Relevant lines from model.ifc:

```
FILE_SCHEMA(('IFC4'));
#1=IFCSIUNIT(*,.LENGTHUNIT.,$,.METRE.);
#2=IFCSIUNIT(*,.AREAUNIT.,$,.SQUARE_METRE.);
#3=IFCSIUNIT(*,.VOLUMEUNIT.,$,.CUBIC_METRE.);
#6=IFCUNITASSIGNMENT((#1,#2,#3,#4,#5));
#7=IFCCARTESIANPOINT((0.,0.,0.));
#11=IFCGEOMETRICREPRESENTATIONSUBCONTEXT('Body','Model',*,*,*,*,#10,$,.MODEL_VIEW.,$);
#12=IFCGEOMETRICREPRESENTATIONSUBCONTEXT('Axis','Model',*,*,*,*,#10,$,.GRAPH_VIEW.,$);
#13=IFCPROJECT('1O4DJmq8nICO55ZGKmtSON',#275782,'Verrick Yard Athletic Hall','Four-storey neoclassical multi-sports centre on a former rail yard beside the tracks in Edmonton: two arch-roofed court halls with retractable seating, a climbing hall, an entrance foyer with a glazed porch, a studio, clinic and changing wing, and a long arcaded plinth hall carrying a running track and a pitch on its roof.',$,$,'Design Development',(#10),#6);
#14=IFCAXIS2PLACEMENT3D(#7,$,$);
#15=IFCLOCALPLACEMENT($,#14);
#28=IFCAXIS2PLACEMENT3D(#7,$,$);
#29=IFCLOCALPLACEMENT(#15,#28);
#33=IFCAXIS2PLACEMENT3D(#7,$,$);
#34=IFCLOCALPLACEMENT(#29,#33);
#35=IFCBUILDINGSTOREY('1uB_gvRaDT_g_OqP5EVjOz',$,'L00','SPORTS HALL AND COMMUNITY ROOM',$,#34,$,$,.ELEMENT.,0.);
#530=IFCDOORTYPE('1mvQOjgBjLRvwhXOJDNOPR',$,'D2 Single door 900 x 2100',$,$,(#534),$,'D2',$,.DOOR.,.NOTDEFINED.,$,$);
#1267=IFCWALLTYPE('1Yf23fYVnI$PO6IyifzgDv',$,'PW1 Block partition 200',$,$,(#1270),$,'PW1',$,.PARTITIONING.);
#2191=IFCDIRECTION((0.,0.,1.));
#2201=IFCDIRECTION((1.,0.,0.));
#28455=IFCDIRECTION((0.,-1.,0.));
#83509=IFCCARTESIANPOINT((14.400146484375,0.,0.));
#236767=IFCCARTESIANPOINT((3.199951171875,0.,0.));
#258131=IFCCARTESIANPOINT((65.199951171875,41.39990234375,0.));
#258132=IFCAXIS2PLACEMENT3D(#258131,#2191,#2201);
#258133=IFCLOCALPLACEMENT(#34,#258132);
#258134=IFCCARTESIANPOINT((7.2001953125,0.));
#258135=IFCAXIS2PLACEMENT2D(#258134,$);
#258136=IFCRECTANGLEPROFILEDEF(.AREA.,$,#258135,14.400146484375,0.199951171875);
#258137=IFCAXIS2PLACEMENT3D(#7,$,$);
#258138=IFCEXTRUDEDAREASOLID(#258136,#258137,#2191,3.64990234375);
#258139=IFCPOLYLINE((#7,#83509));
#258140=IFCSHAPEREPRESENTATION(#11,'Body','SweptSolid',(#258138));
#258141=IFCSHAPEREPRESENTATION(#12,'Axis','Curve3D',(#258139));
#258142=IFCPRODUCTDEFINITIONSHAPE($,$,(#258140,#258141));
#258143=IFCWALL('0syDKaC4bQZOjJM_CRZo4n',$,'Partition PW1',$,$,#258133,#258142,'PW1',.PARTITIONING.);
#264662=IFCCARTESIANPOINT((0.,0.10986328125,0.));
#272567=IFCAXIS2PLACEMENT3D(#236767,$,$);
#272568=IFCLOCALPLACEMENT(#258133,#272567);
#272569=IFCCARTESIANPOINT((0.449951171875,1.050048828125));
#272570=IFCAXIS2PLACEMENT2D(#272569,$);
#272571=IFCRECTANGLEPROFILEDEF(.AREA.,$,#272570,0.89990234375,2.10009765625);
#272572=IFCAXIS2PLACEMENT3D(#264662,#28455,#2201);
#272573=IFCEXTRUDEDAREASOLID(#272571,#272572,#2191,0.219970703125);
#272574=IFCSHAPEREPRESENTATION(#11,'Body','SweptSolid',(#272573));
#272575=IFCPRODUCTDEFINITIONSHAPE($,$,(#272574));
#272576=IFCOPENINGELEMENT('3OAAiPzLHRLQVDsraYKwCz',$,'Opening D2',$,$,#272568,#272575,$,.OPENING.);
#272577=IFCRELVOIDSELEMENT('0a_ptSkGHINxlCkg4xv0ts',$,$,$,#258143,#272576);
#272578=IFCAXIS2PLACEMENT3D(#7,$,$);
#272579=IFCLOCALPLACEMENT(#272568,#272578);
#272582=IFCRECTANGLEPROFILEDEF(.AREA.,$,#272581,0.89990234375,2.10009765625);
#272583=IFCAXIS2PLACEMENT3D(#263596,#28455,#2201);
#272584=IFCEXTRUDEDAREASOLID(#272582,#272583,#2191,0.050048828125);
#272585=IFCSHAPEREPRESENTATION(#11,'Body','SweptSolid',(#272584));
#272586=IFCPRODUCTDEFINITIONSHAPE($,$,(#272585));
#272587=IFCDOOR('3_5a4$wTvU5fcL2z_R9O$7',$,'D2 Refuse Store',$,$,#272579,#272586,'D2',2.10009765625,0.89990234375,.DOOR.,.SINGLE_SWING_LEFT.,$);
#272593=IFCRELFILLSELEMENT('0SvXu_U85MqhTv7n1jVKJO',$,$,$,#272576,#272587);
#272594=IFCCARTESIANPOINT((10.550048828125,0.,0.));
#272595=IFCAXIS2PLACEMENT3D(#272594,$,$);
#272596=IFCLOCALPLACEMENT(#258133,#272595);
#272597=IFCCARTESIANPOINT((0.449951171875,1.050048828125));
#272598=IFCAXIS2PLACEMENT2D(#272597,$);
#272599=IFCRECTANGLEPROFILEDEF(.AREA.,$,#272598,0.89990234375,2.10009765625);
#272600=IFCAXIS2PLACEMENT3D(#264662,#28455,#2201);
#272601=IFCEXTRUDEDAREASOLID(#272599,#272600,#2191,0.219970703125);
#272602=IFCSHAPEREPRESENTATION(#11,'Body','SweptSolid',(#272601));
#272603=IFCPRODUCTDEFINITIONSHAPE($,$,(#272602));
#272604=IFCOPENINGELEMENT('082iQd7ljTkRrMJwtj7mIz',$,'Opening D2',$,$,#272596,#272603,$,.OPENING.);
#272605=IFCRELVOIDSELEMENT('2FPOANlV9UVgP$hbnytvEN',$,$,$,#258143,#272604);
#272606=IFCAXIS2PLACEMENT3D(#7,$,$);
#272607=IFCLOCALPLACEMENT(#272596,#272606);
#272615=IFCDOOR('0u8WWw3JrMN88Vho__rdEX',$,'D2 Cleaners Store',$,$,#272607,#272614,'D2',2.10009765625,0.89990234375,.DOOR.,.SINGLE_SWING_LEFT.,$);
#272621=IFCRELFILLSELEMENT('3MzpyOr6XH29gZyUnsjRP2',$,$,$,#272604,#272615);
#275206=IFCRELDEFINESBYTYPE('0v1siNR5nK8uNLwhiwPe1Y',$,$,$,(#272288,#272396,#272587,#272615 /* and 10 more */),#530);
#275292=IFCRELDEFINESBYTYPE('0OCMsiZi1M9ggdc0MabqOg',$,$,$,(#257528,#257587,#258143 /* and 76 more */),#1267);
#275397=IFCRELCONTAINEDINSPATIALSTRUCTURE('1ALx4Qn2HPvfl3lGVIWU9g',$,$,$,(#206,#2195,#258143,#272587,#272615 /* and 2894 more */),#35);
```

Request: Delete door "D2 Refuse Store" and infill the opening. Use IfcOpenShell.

```python
import ifcopenshell
import ifcopenshell.api.feature
import ifcopenshell.api.root
import ifcopenshell.geom
import ifcopenshell.util.shape

model = ifcopenshell.open("model.ifc")
settings = ifcopenshell.geom.settings()


def volume(element):
    """Net volume in cubic metres, openings subtracted."""
    shape = ifcopenshell.geom.create_shape(settings, element)
    return ifcopenshell.util.shape.get_volume(shape.geometry)


door = model.by_guid("3_5a4$wTvU5fcL2z_R9O$7")
opening = door.FillsVoids[0].RelatingOpeningElement
wall = opening.VoidsElements[0].RelatingBuildingElement
before = volume(wall)

ifcopenshell.api.root.remove_product(model, product=door)
ifcopenshell.api.feature.remove_feature(model, feature=opening)

after = volume(wall)

print(f"wall volume {before:.3f} -> {after:.3f} m3")

model.write("model_edited.ifc")
```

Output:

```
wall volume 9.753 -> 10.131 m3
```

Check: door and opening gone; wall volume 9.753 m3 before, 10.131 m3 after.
